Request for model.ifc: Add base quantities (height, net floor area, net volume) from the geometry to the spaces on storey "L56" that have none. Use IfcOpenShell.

First a look at what the model holds.

```python
import ifcopenshell
import ifcopenshell.util.element
import ifcopenshell.util.unit

model = ifcopenshell.open("model.ifc")
print(model.schema)
for unit_type in ("LENGTHUNIT", "AREAUNIT", "VOLUMEUNIT"):
    print(unit_type, ifcopenshell.util.unit.calculate_unit_scale(model, unit_type))
storey = next(s for s in model.by_type("IfcBuildingStorey") if s.Name == "L56")
spaces = [e for e in ifcopenshell.util.element.get_decomposition(storey) if e.is_a("IfcSpace")]
for e in sorted(spaces, key=lambda e: e.id()):
    print(e.id(), e.is_a(), e.Name, list(ifcopenshell.util.element.get_psets(e, qtos_only=True)), sep=" | ")
```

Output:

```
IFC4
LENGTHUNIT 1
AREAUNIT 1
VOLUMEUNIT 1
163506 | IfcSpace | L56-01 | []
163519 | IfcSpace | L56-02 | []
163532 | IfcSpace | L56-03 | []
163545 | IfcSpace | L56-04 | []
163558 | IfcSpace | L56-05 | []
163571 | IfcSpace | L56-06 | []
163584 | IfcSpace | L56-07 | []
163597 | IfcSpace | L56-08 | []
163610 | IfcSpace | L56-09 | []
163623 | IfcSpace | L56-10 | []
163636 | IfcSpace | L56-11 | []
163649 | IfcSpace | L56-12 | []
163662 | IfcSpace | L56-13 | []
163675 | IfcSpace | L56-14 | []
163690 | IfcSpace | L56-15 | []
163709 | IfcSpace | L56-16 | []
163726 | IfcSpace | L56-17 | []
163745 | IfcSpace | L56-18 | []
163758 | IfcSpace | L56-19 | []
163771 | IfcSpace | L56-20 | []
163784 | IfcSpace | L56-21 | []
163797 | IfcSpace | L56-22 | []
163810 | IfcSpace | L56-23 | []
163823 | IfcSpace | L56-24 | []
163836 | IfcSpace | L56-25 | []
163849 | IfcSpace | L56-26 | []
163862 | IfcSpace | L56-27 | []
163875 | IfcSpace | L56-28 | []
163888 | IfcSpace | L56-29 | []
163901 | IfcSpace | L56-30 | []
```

```python
import ifcopenshell
import ifcopenshell.api.pset
import ifcopenshell.geom
import ifcopenshell.util.element
import ifcopenshell.util.shape
import ifcopenshell.util.unit

model = ifcopenshell.open("model.ifc")
unit_scale = ifcopenshell.util.unit.calculate_unit_scale(model)
area_scale = ifcopenshell.util.unit.calculate_unit_scale(model, "AREAUNIT")
volume_scale = ifcopenshell.util.unit.calculate_unit_scale(model, "VOLUMEUNIT")
settings = ifcopenshell.geom.settings()

storey = next(s for s in model.by_type("IfcBuildingStorey") if s.Name == "L56")
spaces = [e for e in ifcopenshell.util.element.get_decomposition(storey) if e.is_a("IfcSpace")]

for e in sorted(spaces, key=lambda e: e.id()):
    if ifcopenshell.util.element.get_psets(e, qtos_only=True, should_inherit=False):
        continue
    # Geometry comes back in metres, in the element's own axes.
    shape = ifcopenshell.geom.create_shape(settings, e)
    values = {
        "Height": ifcopenshell.util.shape.get_z(shape.geometry) / unit_scale,
        "NetFloorArea": ifcopenshell.util.shape.get_footprint_area(shape.geometry) / area_scale,
        "NetVolume": ifcopenshell.util.shape.get_volume(shape.geometry) / volume_scale,
    }
    qto = ifcopenshell.api.pset.add_qto(model, product=e, name="Qto_SpaceBaseQuantities")
    ifcopenshell.api.pset.edit_qto(model, qto=qto, properties=values)
    print(e.id(), {k: round(v, 3) for k, v in values.items()})

model.write("model_v2.ifc")
```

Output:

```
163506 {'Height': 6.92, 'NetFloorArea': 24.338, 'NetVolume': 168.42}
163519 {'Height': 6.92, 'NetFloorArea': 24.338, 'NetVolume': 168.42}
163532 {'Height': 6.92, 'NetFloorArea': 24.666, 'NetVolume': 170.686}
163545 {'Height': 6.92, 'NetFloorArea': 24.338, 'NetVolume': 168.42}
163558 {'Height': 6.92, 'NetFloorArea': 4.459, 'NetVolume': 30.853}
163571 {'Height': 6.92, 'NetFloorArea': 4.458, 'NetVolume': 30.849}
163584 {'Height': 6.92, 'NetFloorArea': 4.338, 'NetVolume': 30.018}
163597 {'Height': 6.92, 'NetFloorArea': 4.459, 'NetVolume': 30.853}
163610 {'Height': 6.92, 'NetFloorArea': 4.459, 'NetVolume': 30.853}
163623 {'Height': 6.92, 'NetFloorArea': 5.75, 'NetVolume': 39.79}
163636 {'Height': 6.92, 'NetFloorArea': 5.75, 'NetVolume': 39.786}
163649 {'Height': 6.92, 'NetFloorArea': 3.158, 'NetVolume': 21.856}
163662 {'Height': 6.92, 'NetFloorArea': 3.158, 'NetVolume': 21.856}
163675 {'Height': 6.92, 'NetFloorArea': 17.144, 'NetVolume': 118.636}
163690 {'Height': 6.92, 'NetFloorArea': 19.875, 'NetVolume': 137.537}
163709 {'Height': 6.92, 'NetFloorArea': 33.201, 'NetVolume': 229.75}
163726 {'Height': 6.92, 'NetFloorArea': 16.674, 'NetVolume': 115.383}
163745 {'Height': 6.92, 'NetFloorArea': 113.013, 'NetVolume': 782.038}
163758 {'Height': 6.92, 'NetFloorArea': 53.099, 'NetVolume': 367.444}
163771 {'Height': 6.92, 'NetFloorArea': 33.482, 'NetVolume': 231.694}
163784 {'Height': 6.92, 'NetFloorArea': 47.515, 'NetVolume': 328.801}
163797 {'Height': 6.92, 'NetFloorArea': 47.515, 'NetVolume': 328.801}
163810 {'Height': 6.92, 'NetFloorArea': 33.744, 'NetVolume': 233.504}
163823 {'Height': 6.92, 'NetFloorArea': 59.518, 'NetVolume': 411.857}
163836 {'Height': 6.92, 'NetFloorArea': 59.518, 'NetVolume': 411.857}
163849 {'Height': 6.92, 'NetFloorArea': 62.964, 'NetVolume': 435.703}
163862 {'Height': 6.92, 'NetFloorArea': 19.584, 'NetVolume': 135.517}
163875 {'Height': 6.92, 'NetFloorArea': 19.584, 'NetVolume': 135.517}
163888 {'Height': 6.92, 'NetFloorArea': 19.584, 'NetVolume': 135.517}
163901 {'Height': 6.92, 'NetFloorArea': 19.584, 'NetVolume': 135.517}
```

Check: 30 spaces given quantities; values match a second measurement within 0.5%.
